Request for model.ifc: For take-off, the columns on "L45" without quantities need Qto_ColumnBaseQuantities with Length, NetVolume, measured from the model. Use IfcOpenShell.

First a look at what the model holds.

```python
import ifcopenshell
import ifcopenshell.util.element
import ifcopenshell.util.unit

model = ifcopenshell.open("model.ifc")
print(model.schema)
for unit_type in ("LENGTHUNIT", "AREAUNIT", "VOLUMEUNIT"):
    print(unit_type, ifcopenshell.util.unit.calculate_unit_scale(model, unit_type))
storey = next(s for s in model.by_type("IfcBuildingStorey") if s.Name == "L45")
columns = [e for e in ifcopenshell.util.element.get_decomposition(storey) if e.is_a("IfcColumn")]
for e in sorted(columns, key=lambda e: e.id()):
    print(e.id(), e.is_a(), e.Name, list(ifcopenshell.util.element.get_psets(e, qtos_only=True)), sep=" | ")
```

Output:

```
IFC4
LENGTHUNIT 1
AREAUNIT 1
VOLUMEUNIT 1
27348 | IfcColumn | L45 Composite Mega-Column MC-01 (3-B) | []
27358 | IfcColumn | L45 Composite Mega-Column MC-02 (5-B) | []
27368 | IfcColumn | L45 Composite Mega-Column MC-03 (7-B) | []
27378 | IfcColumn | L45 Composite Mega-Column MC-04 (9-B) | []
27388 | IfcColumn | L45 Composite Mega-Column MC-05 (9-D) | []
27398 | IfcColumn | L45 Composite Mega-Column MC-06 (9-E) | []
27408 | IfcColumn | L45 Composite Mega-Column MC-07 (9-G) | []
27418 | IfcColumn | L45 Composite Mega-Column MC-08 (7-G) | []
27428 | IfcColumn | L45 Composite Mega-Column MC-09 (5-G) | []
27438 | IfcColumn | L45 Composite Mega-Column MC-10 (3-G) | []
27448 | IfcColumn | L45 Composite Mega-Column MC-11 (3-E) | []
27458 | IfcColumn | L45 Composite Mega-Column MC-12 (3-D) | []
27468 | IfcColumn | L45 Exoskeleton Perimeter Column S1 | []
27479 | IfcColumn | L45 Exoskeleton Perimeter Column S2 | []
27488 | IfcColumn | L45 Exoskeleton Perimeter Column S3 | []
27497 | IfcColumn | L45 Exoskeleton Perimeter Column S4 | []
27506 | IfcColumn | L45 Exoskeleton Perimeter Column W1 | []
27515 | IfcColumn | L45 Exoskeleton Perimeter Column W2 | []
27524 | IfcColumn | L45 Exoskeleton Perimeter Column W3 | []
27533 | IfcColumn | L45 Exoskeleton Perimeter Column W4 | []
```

```python
import ifcopenshell
import ifcopenshell.api.pset
import ifcopenshell.geom
import ifcopenshell.util.element
import ifcopenshell.util.shape
import ifcopenshell.util.unit

model = ifcopenshell.open("model.ifc")
unit_scale = ifcopenshell.util.unit.calculate_unit_scale(model)
volume_scale = ifcopenshell.util.unit.calculate_unit_scale(model, "VOLUMEUNIT")
settings = ifcopenshell.geom.settings()

storey = next(s for s in model.by_type("IfcBuildingStorey") if s.Name == "L45")
columns = [e for e in ifcopenshell.util.element.get_decomposition(storey) if e.is_a("IfcColumn")]

for e in sorted(columns, key=lambda e: e.id()):
    if ifcopenshell.util.element.get_psets(e, qtos_only=True, should_inherit=False):
        continue
    # Geometry comes back in metres, in the element's own axes.
    shape = ifcopenshell.geom.create_shape(settings, e)
    values = {
        "Length": ifcopenshell.util.shape.get_z(shape.geometry) / unit_scale,
        "NetVolume": ifcopenshell.util.shape.get_volume(shape.geometry) / volume_scale,
    }
    qto = ifcopenshell.api.pset.add_qto(model, product=e, name="Qto_ColumnBaseQuantities")
    ifcopenshell.api.pset.edit_qto(model, qto=qto, properties=values)
    print(e.id(), {k: round(v, 3) for k, v in values.items()})

model.write("model_edited.ifc")
```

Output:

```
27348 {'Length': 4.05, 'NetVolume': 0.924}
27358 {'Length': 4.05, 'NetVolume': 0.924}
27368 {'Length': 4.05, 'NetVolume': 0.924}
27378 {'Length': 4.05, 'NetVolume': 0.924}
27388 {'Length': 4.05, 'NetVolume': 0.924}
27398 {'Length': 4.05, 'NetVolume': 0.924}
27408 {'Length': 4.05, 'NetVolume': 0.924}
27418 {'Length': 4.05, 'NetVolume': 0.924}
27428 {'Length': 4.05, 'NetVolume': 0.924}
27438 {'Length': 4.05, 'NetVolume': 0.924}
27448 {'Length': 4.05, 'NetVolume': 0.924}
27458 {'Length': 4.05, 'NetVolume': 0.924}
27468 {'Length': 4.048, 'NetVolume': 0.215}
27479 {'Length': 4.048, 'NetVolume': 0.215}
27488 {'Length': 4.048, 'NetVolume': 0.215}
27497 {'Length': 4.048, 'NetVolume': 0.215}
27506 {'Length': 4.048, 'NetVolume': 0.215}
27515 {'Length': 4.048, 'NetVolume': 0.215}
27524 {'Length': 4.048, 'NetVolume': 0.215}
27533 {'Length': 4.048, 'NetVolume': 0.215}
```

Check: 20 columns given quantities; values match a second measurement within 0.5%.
